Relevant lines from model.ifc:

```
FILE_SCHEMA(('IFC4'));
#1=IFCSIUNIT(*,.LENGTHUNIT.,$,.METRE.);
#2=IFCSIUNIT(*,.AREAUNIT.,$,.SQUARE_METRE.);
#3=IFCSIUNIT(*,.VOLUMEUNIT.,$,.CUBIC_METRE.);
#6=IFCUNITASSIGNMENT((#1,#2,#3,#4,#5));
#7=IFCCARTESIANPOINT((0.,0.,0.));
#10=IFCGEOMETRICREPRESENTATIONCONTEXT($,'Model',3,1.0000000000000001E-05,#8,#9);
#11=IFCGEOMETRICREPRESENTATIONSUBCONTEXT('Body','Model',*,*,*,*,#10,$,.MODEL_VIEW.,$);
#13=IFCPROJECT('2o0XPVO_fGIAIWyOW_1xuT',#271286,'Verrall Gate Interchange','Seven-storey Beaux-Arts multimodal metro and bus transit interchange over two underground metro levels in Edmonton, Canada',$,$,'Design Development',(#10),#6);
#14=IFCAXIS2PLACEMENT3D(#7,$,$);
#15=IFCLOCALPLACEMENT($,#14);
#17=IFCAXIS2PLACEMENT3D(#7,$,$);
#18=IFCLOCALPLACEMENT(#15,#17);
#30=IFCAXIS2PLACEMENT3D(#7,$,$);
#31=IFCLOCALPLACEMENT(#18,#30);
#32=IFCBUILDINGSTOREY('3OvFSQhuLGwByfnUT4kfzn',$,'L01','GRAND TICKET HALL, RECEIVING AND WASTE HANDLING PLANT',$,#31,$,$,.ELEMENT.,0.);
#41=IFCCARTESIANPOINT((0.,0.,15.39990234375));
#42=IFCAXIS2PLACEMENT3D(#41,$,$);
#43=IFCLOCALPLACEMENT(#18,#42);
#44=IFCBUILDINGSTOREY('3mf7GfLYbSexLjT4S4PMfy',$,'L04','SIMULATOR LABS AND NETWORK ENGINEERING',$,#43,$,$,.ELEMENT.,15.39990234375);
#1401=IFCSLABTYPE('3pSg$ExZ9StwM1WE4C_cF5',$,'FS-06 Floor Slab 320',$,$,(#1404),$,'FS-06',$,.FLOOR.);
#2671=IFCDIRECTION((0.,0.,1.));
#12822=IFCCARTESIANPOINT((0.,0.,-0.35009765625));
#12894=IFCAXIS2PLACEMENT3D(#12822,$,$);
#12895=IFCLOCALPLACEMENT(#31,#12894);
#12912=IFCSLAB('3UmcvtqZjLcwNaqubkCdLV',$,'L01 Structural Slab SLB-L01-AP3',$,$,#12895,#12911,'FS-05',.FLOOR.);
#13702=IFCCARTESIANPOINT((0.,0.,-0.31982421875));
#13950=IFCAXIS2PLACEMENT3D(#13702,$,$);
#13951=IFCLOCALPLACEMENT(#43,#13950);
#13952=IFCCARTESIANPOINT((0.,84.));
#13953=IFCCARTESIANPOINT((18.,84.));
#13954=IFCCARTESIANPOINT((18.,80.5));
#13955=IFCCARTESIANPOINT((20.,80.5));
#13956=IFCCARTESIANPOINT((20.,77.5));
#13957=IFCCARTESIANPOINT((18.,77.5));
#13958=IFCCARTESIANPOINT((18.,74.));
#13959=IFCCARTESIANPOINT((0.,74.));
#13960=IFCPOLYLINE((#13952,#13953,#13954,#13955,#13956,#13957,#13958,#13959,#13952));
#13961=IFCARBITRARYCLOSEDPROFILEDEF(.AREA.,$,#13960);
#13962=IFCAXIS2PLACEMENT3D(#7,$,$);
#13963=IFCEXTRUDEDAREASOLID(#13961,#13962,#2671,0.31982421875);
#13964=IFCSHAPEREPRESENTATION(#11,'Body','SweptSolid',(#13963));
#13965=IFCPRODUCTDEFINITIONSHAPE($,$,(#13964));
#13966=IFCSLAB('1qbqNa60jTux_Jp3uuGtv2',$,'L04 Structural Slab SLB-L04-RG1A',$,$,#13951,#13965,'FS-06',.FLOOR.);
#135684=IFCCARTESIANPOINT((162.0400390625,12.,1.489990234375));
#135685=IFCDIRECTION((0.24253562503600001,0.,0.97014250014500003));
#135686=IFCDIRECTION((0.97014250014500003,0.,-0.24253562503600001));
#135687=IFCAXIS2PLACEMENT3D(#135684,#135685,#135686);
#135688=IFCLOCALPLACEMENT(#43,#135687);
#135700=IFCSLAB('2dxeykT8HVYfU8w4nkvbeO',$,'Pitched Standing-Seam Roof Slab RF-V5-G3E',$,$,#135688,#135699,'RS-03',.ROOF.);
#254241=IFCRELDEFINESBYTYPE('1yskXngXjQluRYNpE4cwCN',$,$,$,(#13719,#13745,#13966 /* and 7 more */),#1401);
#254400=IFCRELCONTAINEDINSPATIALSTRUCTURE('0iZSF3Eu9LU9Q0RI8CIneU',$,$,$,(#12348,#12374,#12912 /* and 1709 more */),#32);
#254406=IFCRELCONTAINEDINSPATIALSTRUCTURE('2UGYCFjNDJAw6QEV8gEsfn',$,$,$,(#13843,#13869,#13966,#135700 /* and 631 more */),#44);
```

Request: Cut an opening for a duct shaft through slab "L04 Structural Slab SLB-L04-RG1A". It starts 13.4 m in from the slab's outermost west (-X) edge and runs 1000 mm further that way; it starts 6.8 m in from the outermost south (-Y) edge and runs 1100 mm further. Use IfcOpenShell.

```python
import numpy as np
import ifcopenshell
import ifcopenshell.api.feature
import ifcopenshell.api.geometry
import ifcopenshell.api.root
import ifcopenshell.geom
import ifcopenshell.util.placement
import ifcopenshell.util.representation
import ifcopenshell.util.shape
import ifcopenshell.util.unit

model = ifcopenshell.open("model.ifc")
unit_scale = ifcopenshell.util.unit.calculate_unit_scale(model)
settings = ifcopenshell.geom.settings()


def volume(element):
    """Net volume in cubic metres, openings subtracted."""
    shape = ifcopenshell.geom.create_shape(settings, element)
    return ifcopenshell.util.shape.get_volume(shape.geometry)


slab = model.by_guid("1qbqNa60jTux_Jp3uuGtv2")
before = volume(slab)

# Extent in the slab's own axes, in metres. The edges named are its -X and -Y sides.
slab_shape = ifcopenshell.geom.create_shape(settings, slab)
vertices = ifcopenshell.util.shape.get_vertices(slab_shape.geometry)
x_min, y_min, bottom = vertices.min(axis=0)
top = vertices[:, 2].max()

opening = ifcopenshell.api.root.create_entity(model, ifc_class="IfcOpeningElement", name="Duct shaft opening", predefined_type="OPENING")
context = ifcopenshell.util.representation.get_context(model, "Model", "Body", "MODEL_VIEW")
width, depth = 1, 1.1
outline = [(0.0, 0.0), (width, 0.0), (width, depth), (0.0, depth), (0.0, 0.0)]
# Overshoot both faces by 50 mm so the cut is clean.
shape = ifcopenshell.api.geometry.add_slab_representation(
    model, context=context, depth=top - bottom + 0.1, polyline=outline
)
ifcopenshell.api.geometry.assign_representation(model, product=opening, representation=shape)

matrix = ifcopenshell.util.placement.get_local_placement(slab.ObjectPlacement)
matrix[:, 3] = matrix @ np.append(np.array([x_min + 13.4, y_min + 6.8, bottom - 0.05]) / unit_scale, 1.0)
ifcopenshell.api.geometry.edit_object_placement(model, product=opening, matrix=matrix, is_si=False)
ifcopenshell.api.feature.add_feature(model, feature=opening, element=slab)

after = volume(slab)

print(f"slab volume {before:.3f} -> {after:.3f} m3")

model.write("model-out.ifc")
```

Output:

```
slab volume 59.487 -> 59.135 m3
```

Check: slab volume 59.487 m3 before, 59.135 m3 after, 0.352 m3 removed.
